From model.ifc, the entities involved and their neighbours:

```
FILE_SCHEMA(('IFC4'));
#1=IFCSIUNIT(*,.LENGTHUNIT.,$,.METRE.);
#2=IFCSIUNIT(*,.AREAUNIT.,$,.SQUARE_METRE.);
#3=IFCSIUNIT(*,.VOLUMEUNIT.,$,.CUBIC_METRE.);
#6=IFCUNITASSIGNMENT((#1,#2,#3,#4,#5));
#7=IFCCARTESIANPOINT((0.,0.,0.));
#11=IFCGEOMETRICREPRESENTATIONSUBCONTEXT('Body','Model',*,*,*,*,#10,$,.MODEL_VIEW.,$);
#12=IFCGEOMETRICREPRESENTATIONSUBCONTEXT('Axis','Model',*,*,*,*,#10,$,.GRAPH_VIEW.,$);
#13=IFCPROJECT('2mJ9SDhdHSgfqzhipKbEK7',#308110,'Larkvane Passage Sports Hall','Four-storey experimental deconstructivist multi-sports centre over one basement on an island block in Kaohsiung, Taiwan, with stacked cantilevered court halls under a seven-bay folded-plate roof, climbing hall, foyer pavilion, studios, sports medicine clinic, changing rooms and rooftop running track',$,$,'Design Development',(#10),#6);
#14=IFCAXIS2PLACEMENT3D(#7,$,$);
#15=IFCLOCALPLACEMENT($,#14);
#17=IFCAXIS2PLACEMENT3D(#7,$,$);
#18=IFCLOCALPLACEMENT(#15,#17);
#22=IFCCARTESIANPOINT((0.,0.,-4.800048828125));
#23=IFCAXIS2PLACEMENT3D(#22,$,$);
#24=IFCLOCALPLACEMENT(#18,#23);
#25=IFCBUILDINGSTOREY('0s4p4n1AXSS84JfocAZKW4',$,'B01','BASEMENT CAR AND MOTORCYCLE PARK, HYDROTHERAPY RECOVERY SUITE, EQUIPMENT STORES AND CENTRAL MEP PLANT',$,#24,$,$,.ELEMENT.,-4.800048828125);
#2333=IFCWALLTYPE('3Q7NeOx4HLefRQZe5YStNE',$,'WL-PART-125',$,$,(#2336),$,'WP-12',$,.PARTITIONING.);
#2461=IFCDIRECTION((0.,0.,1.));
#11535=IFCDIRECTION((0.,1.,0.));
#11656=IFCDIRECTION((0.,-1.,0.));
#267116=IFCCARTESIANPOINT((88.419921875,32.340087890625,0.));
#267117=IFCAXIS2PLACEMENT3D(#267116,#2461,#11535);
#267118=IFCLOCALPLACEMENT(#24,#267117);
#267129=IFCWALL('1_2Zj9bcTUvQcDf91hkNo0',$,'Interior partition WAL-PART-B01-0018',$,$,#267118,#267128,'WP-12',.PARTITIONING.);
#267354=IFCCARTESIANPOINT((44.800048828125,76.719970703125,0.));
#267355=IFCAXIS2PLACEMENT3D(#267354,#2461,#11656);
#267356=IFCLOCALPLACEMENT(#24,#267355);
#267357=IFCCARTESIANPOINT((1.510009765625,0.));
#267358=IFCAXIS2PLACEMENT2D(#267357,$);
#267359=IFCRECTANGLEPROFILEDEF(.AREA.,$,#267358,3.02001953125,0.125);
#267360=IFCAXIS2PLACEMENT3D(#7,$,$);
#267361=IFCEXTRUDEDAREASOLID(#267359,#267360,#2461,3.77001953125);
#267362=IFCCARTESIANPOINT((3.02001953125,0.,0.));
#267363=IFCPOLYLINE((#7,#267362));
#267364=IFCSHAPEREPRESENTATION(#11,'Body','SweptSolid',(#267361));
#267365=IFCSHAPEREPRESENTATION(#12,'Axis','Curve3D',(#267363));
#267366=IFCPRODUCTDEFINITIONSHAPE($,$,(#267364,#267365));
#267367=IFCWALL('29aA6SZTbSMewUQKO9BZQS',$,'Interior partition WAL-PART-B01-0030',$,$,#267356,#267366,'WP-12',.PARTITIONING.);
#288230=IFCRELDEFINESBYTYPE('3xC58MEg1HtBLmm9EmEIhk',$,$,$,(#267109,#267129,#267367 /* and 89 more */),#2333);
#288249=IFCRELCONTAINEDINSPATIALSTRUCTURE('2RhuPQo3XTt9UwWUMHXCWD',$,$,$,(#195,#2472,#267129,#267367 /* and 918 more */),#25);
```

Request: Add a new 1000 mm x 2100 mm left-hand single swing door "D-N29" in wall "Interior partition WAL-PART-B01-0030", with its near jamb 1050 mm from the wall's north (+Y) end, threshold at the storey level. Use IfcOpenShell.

```python
import numpy as np
import ifcopenshell
import ifcopenshell.api.feature
import ifcopenshell.api.geometry
import ifcopenshell.api.root
import ifcopenshell.api.spatial
import ifcopenshell.geom
import ifcopenshell.util.element
import ifcopenshell.util.placement
import ifcopenshell.util.representation
import ifcopenshell.util.shape
import ifcopenshell.util.unit

model = ifcopenshell.open("model.ifc")
unit_scale = ifcopenshell.util.unit.calculate_unit_scale(model)
settings = ifcopenshell.geom.settings()


def volume(element):
    """Net volume in cubic metres, openings subtracted."""
    shape = ifcopenshell.geom.create_shape(settings, element)
    return ifcopenshell.util.shape.get_volume(shape.geometry)


wall = model.by_guid("29aA6SZTbSMewUQKO9BZQS")
storey = ifcopenshell.util.element.get_container(wall, ifc_class="IfcBuildingStorey")
context = ifcopenshell.util.representation.get_context(model, "Model", "Body", "MODEL_VIEW")
before = volume(wall)

width, height, from_end, sill = 1, 2.1, 1.05, 0.0  # metres

# The wall runs along its own X axis, and the end named is its -X end.
wall_shape = ifcopenshell.geom.create_shape(settings, wall)
x, y, z = ifcopenshell.util.shape.get_vertices(wall_shape.geometry).T
start = x.min() + from_end
face, thickness = float(y.min()), float(y.max() - y.min())
wall_matrix = ifcopenshell.util.placement.get_local_placement(wall.ObjectPlacement)
level = ifcopenshell.util.placement.get_local_placement(storey.ObjectPlacement)[2, 3]


def in_wall(x, y):
    """Placement at x, y metres in the wall's axes, at sill height."""
    matrix = wall_matrix.copy()
    matrix[:, 3] = wall_matrix @ np.array([x / unit_scale, y / unit_scale, 0.0, 1.0])
    matrix[2, 3] = level + sill / unit_scale
    return matrix


# Opening: a box that overshoots both wall faces by 50 mm.
opening = ifcopenshell.api.root.create_entity(model, ifc_class="IfcOpeningElement", predefined_type="OPENING")
box = ifcopenshell.api.geometry.add_wall_representation(
    model, context=context, length=width, height=height, thickness=thickness + 0.1
)
ifcopenshell.api.geometry.assign_representation(model, product=opening, representation=box)
ifcopenshell.api.geometry.edit_object_placement(model, product=opening, matrix=in_wall(start, face - 0.05), is_si=False)
ifcopenshell.api.feature.add_feature(model, feature=opening, element=wall)

door = ifcopenshell.api.root.create_entity(model, ifc_class="IfcDoor", name="D-N29", predefined_type="DOOR")
door.OverallWidth, door.OverallHeight = width / unit_scale, height / unit_scale
door.OperationType = "SINGLE_SWING_LEFT"
body = ifcopenshell.api.geometry.add_door_representation(
    model,
    context=context,
    overall_width=door.OverallWidth,
    overall_height=door.OverallHeight,
    operation_type="SINGLE_SWING_LEFT",
    lining_properties={"LiningDepth": thickness / unit_scale, "ThresholdDepth": thickness / unit_scale},
)
ifcopenshell.api.geometry.assign_representation(model, product=door, representation=body)
ifcopenshell.api.spatial.assign_container(model, products=[door], relating_structure=storey)
ifcopenshell.api.feature.add_filling(model, opening=opening, element=door)

# The lining spans the wall, so the door starts at the wall face.
ifcopenshell.api.geometry.edit_object_placement(model, product=door, matrix=in_wall(start, face), is_si=False)

after = volume(wall)

print(f"wall volume {before:.3f} -> {after:.3f} m3")

model.write("model_updated.ifc")
```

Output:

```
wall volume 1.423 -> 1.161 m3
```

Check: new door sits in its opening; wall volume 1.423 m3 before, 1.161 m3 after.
